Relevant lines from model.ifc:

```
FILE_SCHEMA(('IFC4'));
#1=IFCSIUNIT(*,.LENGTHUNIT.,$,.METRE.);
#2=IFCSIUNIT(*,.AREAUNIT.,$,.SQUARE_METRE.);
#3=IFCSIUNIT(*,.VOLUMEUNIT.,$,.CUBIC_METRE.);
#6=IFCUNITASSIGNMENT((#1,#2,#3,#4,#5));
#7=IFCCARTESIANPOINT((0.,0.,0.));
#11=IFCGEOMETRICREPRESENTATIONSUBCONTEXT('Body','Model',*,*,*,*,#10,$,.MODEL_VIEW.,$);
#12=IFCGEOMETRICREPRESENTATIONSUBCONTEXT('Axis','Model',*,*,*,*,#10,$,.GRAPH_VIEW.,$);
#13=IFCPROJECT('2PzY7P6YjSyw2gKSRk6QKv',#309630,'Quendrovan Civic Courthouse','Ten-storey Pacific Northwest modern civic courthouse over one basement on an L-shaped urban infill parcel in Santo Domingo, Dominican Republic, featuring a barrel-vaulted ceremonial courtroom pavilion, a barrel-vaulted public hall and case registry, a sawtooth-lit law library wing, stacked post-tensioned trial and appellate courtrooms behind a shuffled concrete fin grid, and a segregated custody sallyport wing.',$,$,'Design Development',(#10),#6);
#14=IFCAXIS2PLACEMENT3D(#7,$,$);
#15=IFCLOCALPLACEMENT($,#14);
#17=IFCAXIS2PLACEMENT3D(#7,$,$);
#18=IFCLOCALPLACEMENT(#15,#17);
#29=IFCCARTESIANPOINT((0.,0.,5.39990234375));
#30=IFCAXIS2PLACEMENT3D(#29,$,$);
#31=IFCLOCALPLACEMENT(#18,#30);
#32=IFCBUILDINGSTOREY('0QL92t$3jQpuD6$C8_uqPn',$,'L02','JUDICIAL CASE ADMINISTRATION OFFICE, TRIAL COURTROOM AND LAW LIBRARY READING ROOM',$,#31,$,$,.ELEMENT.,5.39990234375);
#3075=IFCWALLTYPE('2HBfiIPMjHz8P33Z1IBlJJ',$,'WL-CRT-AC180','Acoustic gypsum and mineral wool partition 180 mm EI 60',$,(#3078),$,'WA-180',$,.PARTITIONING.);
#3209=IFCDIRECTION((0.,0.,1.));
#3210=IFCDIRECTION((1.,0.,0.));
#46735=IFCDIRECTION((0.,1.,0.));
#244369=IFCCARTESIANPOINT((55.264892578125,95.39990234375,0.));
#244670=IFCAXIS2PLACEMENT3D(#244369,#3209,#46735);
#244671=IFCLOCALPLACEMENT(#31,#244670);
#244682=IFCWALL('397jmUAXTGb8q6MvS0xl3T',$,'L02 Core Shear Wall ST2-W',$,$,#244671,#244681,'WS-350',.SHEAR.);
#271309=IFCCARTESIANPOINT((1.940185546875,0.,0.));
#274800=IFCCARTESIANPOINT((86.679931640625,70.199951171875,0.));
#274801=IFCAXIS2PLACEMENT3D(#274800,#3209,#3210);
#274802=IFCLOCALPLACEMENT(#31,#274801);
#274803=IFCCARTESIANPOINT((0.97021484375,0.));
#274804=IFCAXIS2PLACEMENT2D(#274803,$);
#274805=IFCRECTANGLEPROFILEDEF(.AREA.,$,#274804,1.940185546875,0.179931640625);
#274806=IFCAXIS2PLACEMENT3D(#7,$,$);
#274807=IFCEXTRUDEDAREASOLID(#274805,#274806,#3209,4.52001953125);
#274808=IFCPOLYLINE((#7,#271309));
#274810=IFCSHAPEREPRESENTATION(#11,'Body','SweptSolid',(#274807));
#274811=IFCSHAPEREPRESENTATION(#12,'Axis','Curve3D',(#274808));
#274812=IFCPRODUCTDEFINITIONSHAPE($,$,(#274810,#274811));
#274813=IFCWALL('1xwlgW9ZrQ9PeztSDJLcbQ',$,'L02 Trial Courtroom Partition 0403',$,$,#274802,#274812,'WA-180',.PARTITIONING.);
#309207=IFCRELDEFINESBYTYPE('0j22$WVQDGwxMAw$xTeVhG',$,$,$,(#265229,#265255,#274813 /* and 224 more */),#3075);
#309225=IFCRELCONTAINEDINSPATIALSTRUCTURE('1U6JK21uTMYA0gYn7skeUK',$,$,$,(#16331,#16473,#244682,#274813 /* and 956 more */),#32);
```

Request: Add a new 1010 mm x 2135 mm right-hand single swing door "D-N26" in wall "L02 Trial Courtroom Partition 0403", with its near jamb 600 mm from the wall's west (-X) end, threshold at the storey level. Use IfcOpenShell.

```python
import numpy as np
import ifcopenshell
import ifcopenshell.api.feature
import ifcopenshell.api.geometry
import ifcopenshell.api.root
import ifcopenshell.api.spatial
import ifcopenshell.geom
import ifcopenshell.util.element
import ifcopenshell.util.placement
import ifcopenshell.util.representation
import ifcopenshell.util.shape
import ifcopenshell.util.unit

model = ifcopenshell.open("model.ifc")
unit_scale = ifcopenshell.util.unit.calculate_unit_scale(model)
settings = ifcopenshell.geom.settings()


def volume(element):
    """Net volume in cubic metres, openings subtracted."""
    shape = ifcopenshell.geom.create_shape(settings, element)
    return ifcopenshell.util.shape.get_volume(shape.geometry)


wall = model.by_id(274813)
storey = ifcopenshell.util.element.get_container(wall, ifc_class="IfcBuildingStorey")
context = ifcopenshell.util.representation.get_context(model, "Model", "Body", "MODEL_VIEW")
before = volume(wall)

width, height, from_end, sill = 1.01, 2.135, 0.6, 0.0  # metres

# The wall runs along its own X axis, and the end named is its -X end.
wall_shape = ifcopenshell.geom.create_shape(settings, wall)
x, y, z = ifcopenshell.util.shape.get_vertices(wall_shape.geometry).T
start = x.min() + from_end
face, thickness = float(y.min()), float(y.max() - y.min())
wall_matrix = ifcopenshell.util.placement.get_local_placement(wall.ObjectPlacement)
level = ifcopenshell.util.placement.get_local_placement(storey.ObjectPlacement)[2, 3]


def in_wall(x, y):
    """Placement at x, y metres in the wall's axes, at sill height."""
    matrix = wall_matrix.copy()
    matrix[:, 3] = wall_matrix @ np.array([x / unit_scale, y / unit_scale, 0.0, 1.0])
    matrix[2, 3] = level + sill / unit_scale
    return matrix


# Opening: a box that overshoots both wall faces by 50 mm.
opening = ifcopenshell.api.root.create_entity(model, ifc_class="IfcOpeningElement", predefined_type="OPENING")
box = ifcopenshell.api.geometry.add_wall_representation(
    model, context=context, length=width, height=height, thickness=thickness + 0.1
)
ifcopenshell.api.geometry.assign_representation(model, product=opening, representation=box)
ifcopenshell.api.geometry.edit_object_placement(model, product=opening, matrix=in_wall(start, face - 0.05), is_si=False)
ifcopenshell.api.feature.add_feature(model, feature=opening, element=wall)

door = ifcopenshell.api.root.create_entity(model, ifc_class="IfcDoor", name="D-N26", predefined_type="DOOR")
door.OverallWidth, door.OverallHeight = width / unit_scale, height / unit_scale
door.OperationType = "SINGLE_SWING_RIGHT"
body = ifcopenshell.api.geometry.add_door_representation(
    model,
    context=context,
    overall_width=door.OverallWidth,
    overall_height=door.OverallHeight,
    operation_type="SINGLE_SWING_RIGHT",
    lining_properties={"LiningDepth": thickness / unit_scale, "ThresholdDepth": thickness / unit_scale},
)
ifcopenshell.api.geometry.assign_representation(model, product=door, representation=body)
ifcopenshell.api.spatial.assign_container(model, products=[door], relating_structure=storey)
ifcopenshell.api.feature.add_filling(model, opening=opening, element=door)

# The lining spans the wall, so the door starts at the wall face.
ifcopenshell.api.geometry.edit_object_placement(model, product=door, matrix=in_wall(start, face), is_si=False)

after = volume(wall)

print(f"wall volume {before:.3f} -> {after:.3f} m3")

model.write("model_rev.ifc")
```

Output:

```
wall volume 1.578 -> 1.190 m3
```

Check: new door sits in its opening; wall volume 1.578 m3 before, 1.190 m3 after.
